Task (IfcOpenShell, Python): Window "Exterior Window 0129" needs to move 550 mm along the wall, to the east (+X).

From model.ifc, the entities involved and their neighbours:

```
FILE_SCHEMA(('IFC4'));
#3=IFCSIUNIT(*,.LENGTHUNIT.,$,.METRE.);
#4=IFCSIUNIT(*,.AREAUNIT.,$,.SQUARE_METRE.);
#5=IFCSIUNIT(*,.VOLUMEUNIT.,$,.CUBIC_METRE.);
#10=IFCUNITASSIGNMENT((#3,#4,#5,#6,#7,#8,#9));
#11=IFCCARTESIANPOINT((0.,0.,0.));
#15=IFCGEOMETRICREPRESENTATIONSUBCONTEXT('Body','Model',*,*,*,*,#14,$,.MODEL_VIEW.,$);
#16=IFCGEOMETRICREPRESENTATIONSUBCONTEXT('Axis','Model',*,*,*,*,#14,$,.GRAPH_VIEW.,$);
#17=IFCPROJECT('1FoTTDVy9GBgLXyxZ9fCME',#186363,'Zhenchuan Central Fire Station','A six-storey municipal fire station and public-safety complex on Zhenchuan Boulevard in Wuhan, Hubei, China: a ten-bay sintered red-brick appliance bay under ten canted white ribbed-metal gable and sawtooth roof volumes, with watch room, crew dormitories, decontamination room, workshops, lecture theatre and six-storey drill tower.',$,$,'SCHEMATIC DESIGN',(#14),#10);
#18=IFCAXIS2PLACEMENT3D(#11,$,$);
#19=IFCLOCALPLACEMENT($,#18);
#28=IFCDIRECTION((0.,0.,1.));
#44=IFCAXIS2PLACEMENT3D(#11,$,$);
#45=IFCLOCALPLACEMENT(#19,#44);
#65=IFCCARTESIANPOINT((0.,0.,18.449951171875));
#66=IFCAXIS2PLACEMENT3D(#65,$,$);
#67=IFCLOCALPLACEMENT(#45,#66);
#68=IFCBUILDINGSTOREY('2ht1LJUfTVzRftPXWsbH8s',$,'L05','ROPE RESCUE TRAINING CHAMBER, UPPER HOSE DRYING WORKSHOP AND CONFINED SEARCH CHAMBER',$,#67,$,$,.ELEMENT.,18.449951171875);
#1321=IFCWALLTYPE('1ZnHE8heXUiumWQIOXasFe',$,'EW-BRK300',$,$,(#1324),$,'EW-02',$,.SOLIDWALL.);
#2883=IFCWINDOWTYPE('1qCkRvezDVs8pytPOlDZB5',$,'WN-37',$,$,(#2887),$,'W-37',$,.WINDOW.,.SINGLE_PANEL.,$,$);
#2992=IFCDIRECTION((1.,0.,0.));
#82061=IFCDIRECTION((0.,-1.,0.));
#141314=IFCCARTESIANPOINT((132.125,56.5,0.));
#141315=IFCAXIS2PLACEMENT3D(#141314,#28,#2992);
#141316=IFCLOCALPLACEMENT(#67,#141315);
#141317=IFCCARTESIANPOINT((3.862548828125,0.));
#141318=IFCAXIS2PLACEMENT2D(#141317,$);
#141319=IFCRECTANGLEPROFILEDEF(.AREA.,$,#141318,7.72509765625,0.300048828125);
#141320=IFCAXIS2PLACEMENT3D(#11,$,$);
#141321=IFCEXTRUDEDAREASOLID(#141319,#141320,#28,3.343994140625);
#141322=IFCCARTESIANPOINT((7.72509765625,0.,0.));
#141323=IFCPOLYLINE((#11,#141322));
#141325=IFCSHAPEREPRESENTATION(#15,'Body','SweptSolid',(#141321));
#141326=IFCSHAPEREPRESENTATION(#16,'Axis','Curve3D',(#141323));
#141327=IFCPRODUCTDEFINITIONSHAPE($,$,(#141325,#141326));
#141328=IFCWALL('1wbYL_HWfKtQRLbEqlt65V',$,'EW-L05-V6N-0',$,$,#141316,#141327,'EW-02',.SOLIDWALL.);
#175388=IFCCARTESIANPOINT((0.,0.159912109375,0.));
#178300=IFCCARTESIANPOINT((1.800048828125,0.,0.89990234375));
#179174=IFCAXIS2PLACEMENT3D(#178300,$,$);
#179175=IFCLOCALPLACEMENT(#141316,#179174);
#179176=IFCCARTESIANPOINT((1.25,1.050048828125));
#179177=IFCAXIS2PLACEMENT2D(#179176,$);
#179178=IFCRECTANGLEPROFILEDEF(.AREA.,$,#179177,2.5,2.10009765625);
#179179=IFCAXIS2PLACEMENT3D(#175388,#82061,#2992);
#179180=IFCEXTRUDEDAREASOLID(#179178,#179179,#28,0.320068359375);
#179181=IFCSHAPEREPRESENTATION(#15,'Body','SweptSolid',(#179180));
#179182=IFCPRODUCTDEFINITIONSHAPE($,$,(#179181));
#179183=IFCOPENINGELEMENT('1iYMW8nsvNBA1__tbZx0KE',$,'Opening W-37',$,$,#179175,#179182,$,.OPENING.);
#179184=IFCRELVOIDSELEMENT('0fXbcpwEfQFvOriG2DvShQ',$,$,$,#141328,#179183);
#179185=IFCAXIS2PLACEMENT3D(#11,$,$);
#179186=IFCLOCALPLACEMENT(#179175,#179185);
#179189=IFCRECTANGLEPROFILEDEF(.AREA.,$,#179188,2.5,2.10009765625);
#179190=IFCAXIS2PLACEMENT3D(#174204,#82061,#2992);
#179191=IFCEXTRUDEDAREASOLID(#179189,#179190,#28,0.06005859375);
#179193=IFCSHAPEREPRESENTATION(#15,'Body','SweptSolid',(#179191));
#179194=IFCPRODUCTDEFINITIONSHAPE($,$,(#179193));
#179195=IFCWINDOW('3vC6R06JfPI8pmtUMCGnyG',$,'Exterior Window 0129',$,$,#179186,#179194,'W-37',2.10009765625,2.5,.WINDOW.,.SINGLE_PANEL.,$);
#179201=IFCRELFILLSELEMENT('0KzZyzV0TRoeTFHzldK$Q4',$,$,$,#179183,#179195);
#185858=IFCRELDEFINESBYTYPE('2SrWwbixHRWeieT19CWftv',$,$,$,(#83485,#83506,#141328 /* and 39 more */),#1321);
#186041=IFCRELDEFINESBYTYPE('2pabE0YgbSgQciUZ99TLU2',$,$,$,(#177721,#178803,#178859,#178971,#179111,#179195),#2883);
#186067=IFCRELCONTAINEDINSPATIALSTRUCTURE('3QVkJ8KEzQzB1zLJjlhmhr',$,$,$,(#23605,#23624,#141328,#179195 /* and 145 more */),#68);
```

```python
import ifcopenshell
import ifcopenshell.api.geometry
import ifcopenshell.util.placement
import ifcopenshell.util.unit

model = ifcopenshell.open("model.ifc")
unit_scale = ifcopenshell.util.unit.calculate_unit_scale(model)

window = model.by_id(179195)
opening = window.FillsVoids[0].RelatingOpeningElement
wall = opening.VoidsElements[0].RelatingBuildingElement

wall_matrix = ifcopenshell.util.placement.get_local_placement(wall.ObjectPlacement)
shift = wall_matrix[:3, 0] * 0.55 / unit_scale
before = ifcopenshell.util.placement.get_local_placement(window.ObjectPlacement)[:3, 3].copy()

# The window is placed relative to its opening, so it follows when the opening moves.
matrix = ifcopenshell.util.placement.get_local_placement(opening.ObjectPlacement)
matrix[:3, 3] += shift
ifcopenshell.api.geometry.edit_object_placement(
    model, product=opening, matrix=matrix, is_si=False, should_transform_children=True
)

after = ifcopenshell.util.placement.get_local_placement(window.ObjectPlacement)[:3, 3]
print("window moved by", (after - before).round(3) + 0.0)

model.write("model-out.ifc")
```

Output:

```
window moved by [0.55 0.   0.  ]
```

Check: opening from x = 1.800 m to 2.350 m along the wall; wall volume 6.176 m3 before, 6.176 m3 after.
